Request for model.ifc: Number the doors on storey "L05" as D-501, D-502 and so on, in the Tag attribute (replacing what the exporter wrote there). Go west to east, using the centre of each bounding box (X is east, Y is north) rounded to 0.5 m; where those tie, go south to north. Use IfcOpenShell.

First a look at what the model holds.

```python
import ifcopenshell
import ifcopenshell.util.element
import ifcopenshell.util.placement

model = ifcopenshell.open("model.ifc")
print(model.schema)
storey = next(s for s in model.by_type("IfcBuildingStorey") if s.Name == "L05")
doors = [e for e in ifcopenshell.util.element.get_decomposition(storey) if e.is_a("IfcDoor")]
for e in sorted(doors, key=lambda e: e.id()):
    origin = ifcopenshell.util.placement.get_local_placement(e.ObjectPlacement)[:3, 3]
    print(e.id(), e.Tag, e.Name, origin.round(2) + 0.0, sep=" | ")
```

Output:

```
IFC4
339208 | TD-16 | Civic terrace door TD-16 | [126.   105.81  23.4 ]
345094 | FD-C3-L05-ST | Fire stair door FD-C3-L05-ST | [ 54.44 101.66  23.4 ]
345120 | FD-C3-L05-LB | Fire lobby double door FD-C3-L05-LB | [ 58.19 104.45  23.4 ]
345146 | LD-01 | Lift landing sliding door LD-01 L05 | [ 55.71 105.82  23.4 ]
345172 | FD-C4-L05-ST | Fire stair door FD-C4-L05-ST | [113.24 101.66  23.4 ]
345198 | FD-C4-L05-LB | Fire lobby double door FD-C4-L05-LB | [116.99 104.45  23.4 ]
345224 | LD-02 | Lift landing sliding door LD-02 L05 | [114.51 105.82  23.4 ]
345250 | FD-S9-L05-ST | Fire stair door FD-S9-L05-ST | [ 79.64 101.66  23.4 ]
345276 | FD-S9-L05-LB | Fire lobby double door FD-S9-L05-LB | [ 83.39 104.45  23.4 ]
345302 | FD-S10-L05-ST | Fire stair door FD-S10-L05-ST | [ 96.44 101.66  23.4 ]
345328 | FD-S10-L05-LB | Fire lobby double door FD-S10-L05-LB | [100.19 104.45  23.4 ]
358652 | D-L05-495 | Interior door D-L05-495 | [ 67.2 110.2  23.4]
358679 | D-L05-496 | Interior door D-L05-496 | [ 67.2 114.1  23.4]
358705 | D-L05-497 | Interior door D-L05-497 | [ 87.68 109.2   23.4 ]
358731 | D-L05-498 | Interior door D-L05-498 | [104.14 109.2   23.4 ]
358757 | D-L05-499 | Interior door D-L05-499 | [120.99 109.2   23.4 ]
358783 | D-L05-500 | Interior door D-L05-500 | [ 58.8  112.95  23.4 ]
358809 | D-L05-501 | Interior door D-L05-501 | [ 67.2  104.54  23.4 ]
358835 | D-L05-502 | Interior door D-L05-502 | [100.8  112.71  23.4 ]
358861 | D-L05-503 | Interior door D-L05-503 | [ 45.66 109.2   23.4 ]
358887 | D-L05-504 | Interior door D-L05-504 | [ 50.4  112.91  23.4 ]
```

```python
import ifcopenshell
import ifcopenshell.geom
import ifcopenshell.util.element
import ifcopenshell.util.shape

model = ifcopenshell.open("model.ifc")
settings = ifcopenshell.geom.settings()
settings.set("use-world-coords", True)


def centre(element):
    shape = ifcopenshell.geom.create_shape(settings, element)
    return ifcopenshell.util.shape.get_bbox_centroid(shape.geometry)


storey = next(s for s in model.by_type("IfcBuildingStorey") if s.Name == "L05")
doors = [e for e in ifcopenshell.util.element.get_decomposition(storey) if e.is_a("IfcDoor")]

# Insertion points can sit at a corner or the storey origin, so sort by the geometry (in metres).
centres = {e: centre(e) for e in doors}
doors.sort(key=lambda e: (round(centres[e][0] / 0.5), centres[e][1]))

for i, e in enumerate(doors, start=1):
    number = f"D-5{i:02d}"
    e.Tag = number
    print(e.id(), number)

model.write("model_edited.ifc")
```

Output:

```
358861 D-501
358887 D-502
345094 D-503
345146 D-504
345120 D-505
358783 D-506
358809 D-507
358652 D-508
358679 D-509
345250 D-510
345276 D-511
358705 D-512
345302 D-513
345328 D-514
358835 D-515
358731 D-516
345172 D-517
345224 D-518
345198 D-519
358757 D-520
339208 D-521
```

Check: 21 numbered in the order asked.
